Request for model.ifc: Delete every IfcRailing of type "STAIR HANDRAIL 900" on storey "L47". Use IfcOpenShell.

First a look at what the model holds.

```python
import ifcopenshell
import ifcopenshell.util.element

model = ifcopenshell.open("model.ifc")
print(model.schema)
storey = next(s for s in model.by_type("IfcBuildingStorey") if s.Name == "L47")
railings = [e for e in ifcopenshell.util.element.get_decomposition(storey) if e.is_a("IfcRailing")]
seen = {}
for e in railings:
    element_type = ifcopenshell.util.element.get_type(e)
    name = element_type.Name if element_type not in (None, e) else None
    seen[name] = seen.get(name, 0) + 1
for name, count in sorted(seen.items(), key=str):
    print(count, "x", name)
```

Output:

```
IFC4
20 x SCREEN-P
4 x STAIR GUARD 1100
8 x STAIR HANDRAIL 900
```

```python
import ifcopenshell
import ifcopenshell.api.root
import ifcopenshell.util.element

model = ifcopenshell.open("model.ifc")

storey = next(s for s in model.by_type("IfcBuildingStorey") if s.Name == "L47")
railings = [e for e in ifcopenshell.util.element.get_decomposition(storey) if e.is_a("IfcRailing")]
targets = [e for e in railings if (t := ifcopenshell.util.element.get_type(e)) not in (None, e) and t.Name == "STAIR HANDRAIL 900"]

for e in targets:
    ifcopenshell.api.root.remove_product(model, product=e)
print(len(targets), "removed")

model.write("model_edited.ifc")
```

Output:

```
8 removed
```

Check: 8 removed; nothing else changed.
